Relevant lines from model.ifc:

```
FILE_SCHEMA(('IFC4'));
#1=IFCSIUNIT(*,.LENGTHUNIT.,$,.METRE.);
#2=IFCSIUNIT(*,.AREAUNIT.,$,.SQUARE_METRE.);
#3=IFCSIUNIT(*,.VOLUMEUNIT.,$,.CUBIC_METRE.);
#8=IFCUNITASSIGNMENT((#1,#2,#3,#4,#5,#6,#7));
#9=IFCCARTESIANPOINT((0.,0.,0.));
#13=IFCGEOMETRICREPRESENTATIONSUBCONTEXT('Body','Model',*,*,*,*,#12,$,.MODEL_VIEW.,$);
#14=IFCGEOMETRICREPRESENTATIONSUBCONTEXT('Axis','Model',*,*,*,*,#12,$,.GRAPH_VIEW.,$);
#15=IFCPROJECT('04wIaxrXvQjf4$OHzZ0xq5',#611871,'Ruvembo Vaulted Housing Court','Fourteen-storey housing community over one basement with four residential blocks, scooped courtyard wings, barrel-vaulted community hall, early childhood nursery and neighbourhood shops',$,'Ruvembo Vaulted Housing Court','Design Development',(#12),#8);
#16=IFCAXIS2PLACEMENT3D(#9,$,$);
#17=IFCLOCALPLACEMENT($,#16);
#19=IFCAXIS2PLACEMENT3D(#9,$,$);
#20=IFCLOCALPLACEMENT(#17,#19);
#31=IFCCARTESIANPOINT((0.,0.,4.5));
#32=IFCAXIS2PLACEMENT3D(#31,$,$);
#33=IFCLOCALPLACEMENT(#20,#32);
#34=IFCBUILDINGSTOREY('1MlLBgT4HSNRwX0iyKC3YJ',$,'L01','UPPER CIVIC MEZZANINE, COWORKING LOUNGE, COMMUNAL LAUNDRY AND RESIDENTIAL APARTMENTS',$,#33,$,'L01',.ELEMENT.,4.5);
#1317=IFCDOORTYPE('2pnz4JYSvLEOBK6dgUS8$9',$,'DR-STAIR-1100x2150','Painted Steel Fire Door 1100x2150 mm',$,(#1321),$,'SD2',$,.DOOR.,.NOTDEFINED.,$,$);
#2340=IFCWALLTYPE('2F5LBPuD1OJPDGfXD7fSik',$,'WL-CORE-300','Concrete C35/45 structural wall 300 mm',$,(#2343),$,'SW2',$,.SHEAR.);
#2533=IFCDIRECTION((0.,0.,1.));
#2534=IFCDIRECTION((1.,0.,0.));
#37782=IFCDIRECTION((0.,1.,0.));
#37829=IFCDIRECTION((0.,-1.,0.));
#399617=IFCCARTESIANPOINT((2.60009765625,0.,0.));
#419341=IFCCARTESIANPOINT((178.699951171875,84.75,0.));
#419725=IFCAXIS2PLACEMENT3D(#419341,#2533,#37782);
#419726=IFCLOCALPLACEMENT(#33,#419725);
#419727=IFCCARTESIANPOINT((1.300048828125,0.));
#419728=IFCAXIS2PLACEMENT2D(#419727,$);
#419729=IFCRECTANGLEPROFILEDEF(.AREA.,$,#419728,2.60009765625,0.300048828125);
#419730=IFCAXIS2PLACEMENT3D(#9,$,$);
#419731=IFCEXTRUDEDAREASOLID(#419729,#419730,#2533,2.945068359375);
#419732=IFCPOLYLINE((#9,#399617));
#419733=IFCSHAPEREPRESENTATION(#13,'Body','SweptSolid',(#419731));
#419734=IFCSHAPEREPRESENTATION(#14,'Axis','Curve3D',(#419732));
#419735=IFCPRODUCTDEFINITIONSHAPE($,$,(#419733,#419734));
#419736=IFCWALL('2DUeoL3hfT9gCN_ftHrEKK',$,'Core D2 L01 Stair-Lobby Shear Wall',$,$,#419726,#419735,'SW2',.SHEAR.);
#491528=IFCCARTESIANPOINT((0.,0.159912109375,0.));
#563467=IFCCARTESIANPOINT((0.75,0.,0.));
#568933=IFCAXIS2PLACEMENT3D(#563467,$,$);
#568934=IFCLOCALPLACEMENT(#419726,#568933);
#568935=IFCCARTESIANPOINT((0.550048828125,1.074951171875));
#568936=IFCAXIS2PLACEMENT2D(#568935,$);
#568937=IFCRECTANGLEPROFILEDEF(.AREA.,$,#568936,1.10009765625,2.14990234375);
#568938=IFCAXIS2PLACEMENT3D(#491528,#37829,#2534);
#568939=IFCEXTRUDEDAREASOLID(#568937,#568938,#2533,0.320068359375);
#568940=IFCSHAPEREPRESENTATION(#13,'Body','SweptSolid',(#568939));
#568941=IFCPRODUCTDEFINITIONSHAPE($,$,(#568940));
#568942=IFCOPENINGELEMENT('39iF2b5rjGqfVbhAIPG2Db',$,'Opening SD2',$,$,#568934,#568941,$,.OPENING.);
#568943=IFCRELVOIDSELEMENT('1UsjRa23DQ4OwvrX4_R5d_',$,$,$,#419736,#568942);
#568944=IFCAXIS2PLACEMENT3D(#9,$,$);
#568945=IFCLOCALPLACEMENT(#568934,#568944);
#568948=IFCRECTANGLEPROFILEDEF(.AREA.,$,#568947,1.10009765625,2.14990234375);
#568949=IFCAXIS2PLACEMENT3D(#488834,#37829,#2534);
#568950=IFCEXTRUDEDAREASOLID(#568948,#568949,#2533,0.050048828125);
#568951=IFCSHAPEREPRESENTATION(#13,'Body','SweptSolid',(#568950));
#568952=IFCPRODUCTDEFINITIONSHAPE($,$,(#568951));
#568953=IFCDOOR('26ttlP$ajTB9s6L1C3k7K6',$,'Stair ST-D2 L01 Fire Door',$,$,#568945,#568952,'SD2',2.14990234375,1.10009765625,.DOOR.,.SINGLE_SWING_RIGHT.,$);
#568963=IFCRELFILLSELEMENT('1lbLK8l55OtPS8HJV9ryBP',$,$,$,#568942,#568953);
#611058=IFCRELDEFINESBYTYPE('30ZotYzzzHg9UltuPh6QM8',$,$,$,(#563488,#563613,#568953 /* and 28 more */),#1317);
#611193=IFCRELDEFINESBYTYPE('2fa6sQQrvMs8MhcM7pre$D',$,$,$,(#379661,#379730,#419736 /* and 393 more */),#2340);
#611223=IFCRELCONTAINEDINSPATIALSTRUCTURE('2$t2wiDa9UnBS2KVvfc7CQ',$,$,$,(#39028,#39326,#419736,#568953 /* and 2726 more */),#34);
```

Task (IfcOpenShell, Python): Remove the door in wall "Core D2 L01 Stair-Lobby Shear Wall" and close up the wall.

```python
import ifcopenshell
import ifcopenshell.api.feature
import ifcopenshell.api.root
import ifcopenshell.geom
import ifcopenshell.util.shape

model = ifcopenshell.open("model.ifc")
settings = ifcopenshell.geom.settings()


def volume(element):
    """Net volume in cubic metres, openings subtracted."""
    shape = ifcopenshell.geom.create_shape(settings, element)
    return ifcopenshell.util.shape.get_volume(shape.geometry)


door = model.by_guid("26ttlP$ajTB9s6L1C3k7K6")
opening = door.FillsVoids[0].RelatingOpeningElement
wall = opening.VoidsElements[0].RelatingBuildingElement
before = volume(wall)

ifcopenshell.api.root.remove_product(model, product=door)
ifcopenshell.api.feature.remove_feature(model, feature=opening)

after = volume(wall)

print(f"wall volume {before:.3f} -> {after:.3f} m3")

model.write("model-out.ifc")
```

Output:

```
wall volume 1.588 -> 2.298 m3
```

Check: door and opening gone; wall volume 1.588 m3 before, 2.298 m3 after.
